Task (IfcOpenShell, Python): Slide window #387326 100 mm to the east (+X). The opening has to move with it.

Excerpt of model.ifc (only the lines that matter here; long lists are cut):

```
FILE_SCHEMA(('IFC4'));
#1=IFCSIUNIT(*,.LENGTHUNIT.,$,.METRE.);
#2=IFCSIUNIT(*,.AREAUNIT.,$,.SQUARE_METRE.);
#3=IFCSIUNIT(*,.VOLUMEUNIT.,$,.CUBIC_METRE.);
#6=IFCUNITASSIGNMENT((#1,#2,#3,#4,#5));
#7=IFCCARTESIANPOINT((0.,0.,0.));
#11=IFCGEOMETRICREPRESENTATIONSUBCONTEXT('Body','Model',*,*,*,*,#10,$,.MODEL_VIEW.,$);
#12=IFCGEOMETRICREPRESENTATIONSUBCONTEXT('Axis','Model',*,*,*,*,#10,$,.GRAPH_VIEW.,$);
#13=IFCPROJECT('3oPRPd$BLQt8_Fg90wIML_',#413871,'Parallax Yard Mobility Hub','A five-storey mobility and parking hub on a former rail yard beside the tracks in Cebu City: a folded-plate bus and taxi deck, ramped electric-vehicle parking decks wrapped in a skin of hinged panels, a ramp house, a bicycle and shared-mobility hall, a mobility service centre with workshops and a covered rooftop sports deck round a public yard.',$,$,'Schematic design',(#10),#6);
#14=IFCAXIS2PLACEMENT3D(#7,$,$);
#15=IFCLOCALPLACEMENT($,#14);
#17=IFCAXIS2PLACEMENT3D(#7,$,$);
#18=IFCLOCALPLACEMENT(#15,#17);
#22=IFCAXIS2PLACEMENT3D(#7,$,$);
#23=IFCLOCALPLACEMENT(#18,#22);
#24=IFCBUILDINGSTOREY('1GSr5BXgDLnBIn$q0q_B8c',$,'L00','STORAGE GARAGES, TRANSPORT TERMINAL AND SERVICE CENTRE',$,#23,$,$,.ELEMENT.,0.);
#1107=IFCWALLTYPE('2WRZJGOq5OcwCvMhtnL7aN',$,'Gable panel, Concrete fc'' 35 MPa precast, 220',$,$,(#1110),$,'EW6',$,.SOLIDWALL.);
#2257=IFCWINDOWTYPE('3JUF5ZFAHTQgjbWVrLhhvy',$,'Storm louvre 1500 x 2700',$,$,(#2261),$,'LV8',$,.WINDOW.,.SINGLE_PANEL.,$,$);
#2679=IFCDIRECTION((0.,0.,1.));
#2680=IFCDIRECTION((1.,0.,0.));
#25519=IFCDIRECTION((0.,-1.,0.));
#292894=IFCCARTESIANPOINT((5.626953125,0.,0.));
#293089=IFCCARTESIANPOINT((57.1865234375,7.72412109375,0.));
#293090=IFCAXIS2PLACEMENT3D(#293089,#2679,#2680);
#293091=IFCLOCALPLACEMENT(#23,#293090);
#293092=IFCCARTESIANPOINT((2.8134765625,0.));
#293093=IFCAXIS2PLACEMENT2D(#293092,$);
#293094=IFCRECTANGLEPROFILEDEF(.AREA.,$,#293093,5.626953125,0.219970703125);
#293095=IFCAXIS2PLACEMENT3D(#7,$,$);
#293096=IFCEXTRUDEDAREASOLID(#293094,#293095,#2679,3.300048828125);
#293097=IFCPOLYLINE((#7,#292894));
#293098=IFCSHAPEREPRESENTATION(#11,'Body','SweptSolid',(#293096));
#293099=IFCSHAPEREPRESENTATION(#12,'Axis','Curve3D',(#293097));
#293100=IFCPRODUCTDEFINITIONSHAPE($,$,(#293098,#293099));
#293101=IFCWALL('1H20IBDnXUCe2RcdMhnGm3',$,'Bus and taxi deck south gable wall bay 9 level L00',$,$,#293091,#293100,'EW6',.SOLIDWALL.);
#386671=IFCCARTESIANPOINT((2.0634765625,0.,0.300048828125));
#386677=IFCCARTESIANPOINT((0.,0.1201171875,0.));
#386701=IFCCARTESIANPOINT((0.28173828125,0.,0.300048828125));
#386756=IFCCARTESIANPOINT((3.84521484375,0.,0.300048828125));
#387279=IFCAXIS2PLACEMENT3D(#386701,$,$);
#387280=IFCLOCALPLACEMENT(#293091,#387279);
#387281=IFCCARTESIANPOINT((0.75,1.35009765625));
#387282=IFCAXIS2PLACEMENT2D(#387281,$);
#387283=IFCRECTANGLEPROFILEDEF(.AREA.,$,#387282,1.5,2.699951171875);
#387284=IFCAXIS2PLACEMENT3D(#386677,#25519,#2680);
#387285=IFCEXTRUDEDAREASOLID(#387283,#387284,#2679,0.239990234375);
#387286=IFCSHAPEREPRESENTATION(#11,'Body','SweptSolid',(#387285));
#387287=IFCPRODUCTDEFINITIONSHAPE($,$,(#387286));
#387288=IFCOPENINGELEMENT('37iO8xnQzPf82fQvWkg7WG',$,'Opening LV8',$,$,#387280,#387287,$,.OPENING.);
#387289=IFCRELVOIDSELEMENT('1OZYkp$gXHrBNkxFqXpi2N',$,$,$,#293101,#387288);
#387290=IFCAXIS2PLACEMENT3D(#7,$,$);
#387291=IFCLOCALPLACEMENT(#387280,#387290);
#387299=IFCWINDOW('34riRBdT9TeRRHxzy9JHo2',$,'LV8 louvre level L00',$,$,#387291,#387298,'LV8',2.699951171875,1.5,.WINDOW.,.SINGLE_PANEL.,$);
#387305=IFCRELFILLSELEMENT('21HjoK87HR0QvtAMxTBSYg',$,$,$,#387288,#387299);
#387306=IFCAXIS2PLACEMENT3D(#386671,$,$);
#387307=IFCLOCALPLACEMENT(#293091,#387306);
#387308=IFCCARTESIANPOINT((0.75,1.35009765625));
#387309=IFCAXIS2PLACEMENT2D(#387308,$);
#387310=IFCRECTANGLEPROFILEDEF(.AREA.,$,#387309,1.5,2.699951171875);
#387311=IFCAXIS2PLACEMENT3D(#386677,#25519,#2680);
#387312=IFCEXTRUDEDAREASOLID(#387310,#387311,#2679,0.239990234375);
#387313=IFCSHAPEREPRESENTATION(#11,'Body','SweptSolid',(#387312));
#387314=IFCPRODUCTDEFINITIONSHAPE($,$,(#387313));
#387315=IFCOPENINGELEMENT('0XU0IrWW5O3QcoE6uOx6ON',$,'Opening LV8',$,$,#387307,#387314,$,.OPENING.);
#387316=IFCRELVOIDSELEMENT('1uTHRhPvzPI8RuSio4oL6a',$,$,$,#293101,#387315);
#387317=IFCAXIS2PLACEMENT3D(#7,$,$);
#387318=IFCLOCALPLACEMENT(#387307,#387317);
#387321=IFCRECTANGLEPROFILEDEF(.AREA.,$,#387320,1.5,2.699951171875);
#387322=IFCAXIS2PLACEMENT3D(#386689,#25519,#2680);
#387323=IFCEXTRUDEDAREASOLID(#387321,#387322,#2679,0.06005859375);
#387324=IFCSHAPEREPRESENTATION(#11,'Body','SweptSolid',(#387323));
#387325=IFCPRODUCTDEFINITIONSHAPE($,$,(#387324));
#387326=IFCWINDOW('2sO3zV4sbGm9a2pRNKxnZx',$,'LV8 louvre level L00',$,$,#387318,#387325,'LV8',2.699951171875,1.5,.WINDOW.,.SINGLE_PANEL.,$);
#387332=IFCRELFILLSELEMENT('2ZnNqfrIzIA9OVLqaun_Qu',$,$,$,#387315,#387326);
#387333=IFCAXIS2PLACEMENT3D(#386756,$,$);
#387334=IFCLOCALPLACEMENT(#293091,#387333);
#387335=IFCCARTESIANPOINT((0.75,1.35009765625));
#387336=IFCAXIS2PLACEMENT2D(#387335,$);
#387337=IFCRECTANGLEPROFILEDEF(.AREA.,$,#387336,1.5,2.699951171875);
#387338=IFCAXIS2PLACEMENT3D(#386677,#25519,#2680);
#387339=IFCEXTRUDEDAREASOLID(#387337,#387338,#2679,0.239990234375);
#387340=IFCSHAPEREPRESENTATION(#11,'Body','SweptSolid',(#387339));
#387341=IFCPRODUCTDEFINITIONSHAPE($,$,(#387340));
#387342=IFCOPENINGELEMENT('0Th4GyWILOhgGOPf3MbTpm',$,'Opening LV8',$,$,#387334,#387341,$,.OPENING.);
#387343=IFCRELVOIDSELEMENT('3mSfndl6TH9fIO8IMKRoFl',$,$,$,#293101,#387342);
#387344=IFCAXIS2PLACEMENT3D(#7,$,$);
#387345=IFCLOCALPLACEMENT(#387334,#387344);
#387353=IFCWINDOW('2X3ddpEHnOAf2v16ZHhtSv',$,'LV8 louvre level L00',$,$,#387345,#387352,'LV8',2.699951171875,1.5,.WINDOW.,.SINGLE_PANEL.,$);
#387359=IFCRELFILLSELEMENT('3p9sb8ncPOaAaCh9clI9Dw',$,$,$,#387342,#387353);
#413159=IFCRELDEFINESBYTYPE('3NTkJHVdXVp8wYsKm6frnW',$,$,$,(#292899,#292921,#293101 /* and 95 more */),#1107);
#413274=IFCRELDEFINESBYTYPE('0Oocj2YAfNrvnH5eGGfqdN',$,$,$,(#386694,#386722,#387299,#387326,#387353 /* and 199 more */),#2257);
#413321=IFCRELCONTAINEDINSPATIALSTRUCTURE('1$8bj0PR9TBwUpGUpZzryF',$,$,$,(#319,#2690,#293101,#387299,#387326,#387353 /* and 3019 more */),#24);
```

```python
import ifcopenshell
import ifcopenshell.api.geometry
import ifcopenshell.util.placement
import ifcopenshell.util.unit

model = ifcopenshell.open("model.ifc")
unit_scale = ifcopenshell.util.unit.calculate_unit_scale(model)

window = model.by_guid("2sO3zV4sbGm9a2pRNKxnZx")
opening = window.FillsVoids[0].RelatingOpeningElement
wall = opening.VoidsElements[0].RelatingBuildingElement

wall_matrix = ifcopenshell.util.placement.get_local_placement(wall.ObjectPlacement)
shift = wall_matrix[:3, 0] * 0.1 / unit_scale
before = ifcopenshell.util.placement.get_local_placement(window.ObjectPlacement)[:3, 3].copy()

# The window is placed relative to its opening, so it follows when the opening moves.
matrix = ifcopenshell.util.placement.get_local_placement(opening.ObjectPlacement)
matrix[:3, 3] += shift
ifcopenshell.api.geometry.edit_object_placement(
    model, product=opening, matrix=matrix, is_si=False, should_transform_children=True
)

after = ifcopenshell.util.placement.get_local_placement(window.ObjectPlacement)[:3, 3]
print("window moved by", (after - before).round(3) + 0.0)

model.write("model_v2.ifc")
```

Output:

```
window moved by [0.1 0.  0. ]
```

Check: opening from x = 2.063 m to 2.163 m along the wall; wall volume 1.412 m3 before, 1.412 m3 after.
